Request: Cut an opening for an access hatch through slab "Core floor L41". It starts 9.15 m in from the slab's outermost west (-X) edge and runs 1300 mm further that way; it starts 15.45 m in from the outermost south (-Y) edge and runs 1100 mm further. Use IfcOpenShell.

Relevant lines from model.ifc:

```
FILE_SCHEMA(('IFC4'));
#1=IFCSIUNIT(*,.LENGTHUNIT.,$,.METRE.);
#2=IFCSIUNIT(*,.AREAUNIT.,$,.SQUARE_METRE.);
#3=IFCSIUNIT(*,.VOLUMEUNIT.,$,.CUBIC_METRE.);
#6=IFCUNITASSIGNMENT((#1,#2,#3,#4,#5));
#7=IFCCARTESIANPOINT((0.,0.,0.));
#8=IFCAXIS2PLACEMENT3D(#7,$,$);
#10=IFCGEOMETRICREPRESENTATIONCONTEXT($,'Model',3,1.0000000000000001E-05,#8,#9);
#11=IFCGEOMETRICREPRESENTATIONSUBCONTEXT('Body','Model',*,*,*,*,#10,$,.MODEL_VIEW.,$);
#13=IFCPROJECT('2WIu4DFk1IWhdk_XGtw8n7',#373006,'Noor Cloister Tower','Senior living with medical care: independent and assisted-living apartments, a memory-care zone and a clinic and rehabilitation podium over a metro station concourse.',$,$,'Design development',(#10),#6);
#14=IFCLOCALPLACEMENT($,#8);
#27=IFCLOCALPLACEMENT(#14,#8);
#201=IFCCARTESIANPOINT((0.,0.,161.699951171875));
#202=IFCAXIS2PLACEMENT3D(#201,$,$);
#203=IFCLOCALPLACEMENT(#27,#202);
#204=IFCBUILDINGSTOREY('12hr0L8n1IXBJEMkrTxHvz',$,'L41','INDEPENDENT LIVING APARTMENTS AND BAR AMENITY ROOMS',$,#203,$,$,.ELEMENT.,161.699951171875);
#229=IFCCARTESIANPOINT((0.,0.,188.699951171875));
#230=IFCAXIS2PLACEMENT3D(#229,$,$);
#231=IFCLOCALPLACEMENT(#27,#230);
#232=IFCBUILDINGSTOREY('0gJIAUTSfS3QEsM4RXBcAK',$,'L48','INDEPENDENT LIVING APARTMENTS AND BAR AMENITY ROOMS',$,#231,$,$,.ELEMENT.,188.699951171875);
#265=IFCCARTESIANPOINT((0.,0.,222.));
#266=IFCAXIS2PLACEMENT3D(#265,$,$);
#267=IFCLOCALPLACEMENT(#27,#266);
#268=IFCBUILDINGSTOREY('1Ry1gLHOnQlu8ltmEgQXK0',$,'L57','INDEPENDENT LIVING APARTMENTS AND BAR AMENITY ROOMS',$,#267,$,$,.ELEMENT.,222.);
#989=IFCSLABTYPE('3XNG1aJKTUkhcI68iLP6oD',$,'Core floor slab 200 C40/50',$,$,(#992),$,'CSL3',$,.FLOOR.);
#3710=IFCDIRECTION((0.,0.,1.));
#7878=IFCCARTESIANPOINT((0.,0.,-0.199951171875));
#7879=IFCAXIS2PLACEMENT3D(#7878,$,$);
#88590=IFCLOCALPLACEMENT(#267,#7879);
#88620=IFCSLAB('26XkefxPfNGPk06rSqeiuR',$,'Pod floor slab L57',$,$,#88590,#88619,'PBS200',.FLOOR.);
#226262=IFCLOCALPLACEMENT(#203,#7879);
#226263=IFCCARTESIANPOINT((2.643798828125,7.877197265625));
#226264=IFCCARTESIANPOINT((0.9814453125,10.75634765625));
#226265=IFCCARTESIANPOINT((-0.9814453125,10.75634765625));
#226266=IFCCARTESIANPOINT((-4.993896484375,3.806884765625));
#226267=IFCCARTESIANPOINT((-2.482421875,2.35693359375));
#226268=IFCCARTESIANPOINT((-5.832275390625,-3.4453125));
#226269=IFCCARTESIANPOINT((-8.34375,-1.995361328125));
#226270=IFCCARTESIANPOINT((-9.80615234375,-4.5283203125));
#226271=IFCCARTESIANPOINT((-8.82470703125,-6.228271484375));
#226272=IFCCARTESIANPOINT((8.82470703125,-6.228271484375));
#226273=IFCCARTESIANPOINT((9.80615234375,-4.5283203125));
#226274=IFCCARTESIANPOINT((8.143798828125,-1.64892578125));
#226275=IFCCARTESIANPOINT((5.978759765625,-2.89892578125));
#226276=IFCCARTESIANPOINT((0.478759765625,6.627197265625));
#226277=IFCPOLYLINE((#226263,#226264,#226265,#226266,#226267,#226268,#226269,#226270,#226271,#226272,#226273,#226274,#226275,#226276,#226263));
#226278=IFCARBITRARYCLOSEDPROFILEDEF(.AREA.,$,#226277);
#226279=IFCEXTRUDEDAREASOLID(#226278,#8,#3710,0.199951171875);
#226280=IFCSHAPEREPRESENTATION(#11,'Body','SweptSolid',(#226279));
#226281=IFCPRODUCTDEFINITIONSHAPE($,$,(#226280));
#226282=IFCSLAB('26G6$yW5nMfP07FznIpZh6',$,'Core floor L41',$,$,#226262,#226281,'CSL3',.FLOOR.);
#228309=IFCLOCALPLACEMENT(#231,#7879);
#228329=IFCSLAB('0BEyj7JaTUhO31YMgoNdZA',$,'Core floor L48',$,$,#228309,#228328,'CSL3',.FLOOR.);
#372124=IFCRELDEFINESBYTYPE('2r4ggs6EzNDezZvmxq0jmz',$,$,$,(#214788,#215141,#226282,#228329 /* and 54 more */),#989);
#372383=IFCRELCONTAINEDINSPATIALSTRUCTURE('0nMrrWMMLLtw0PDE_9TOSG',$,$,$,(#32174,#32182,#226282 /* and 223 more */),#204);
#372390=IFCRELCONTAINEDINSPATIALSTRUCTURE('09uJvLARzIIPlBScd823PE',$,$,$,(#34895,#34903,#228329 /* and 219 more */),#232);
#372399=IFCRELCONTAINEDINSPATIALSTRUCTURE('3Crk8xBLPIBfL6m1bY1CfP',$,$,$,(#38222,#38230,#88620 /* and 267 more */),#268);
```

```python
import numpy as np
import ifcopenshell
import ifcopenshell.api.feature
import ifcopenshell.api.geometry
import ifcopenshell.api.root
import ifcopenshell.geom
import ifcopenshell.util.placement
import ifcopenshell.util.representation
import ifcopenshell.util.shape
import ifcopenshell.util.unit

model = ifcopenshell.open("model.ifc")
unit_scale = ifcopenshell.util.unit.calculate_unit_scale(model)
settings = ifcopenshell.geom.settings()


def volume(element):
    """Net volume in cubic metres, openings subtracted."""
    shape = ifcopenshell.geom.create_shape(settings, element)
    return ifcopenshell.util.shape.get_volume(shape.geometry)


slab = model.by_guid("26G6$yW5nMfP07FznIpZh6")
before = volume(slab)

# Extent in the slab's own axes, in metres. The edges named are its -X and -Y sides.
slab_shape = ifcopenshell.geom.create_shape(settings, slab)
vertices = ifcopenshell.util.shape.get_vertices(slab_shape.geometry)
x_min, y_min, bottom = vertices.min(axis=0)
top = vertices[:, 2].max()

opening = ifcopenshell.api.root.create_entity(model, ifc_class="IfcOpeningElement", name="Access hatch opening", predefined_type="OPENING")
context = ifcopenshell.util.representation.get_context(model, "Model", "Body", "MODEL_VIEW")
width, depth = 1.3, 1.1
outline = [(0.0, 0.0), (width, 0.0), (width, depth), (0.0, depth), (0.0, 0.0)]
# Overshoot both faces by 50 mm so the cut is clean.
shape = ifcopenshell.api.geometry.add_slab_representation(
    model, context=context, depth=top - bottom + 0.1, polyline=outline
)
ifcopenshell.api.geometry.assign_representation(model, product=opening, representation=shape)

matrix = ifcopenshell.util.placement.get_local_placement(slab.ObjectPlacement)
matrix[:, 3] = matrix @ np.append(np.array([x_min + 9.15, y_min + 15.45, bottom - 0.05]) / unit_scale, 1.0)
ifcopenshell.api.geometry.edit_object_placement(model, product=opening, matrix=matrix, is_si=False)
ifcopenshell.api.feature.add_feature(model, feature=opening, element=slab)

after = volume(slab)

print(f"slab volume {before:.3f} -> {after:.3f} m3")

model.write("model_updated.ifc")
```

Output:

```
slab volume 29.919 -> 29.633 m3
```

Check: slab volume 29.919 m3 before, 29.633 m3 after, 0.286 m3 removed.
